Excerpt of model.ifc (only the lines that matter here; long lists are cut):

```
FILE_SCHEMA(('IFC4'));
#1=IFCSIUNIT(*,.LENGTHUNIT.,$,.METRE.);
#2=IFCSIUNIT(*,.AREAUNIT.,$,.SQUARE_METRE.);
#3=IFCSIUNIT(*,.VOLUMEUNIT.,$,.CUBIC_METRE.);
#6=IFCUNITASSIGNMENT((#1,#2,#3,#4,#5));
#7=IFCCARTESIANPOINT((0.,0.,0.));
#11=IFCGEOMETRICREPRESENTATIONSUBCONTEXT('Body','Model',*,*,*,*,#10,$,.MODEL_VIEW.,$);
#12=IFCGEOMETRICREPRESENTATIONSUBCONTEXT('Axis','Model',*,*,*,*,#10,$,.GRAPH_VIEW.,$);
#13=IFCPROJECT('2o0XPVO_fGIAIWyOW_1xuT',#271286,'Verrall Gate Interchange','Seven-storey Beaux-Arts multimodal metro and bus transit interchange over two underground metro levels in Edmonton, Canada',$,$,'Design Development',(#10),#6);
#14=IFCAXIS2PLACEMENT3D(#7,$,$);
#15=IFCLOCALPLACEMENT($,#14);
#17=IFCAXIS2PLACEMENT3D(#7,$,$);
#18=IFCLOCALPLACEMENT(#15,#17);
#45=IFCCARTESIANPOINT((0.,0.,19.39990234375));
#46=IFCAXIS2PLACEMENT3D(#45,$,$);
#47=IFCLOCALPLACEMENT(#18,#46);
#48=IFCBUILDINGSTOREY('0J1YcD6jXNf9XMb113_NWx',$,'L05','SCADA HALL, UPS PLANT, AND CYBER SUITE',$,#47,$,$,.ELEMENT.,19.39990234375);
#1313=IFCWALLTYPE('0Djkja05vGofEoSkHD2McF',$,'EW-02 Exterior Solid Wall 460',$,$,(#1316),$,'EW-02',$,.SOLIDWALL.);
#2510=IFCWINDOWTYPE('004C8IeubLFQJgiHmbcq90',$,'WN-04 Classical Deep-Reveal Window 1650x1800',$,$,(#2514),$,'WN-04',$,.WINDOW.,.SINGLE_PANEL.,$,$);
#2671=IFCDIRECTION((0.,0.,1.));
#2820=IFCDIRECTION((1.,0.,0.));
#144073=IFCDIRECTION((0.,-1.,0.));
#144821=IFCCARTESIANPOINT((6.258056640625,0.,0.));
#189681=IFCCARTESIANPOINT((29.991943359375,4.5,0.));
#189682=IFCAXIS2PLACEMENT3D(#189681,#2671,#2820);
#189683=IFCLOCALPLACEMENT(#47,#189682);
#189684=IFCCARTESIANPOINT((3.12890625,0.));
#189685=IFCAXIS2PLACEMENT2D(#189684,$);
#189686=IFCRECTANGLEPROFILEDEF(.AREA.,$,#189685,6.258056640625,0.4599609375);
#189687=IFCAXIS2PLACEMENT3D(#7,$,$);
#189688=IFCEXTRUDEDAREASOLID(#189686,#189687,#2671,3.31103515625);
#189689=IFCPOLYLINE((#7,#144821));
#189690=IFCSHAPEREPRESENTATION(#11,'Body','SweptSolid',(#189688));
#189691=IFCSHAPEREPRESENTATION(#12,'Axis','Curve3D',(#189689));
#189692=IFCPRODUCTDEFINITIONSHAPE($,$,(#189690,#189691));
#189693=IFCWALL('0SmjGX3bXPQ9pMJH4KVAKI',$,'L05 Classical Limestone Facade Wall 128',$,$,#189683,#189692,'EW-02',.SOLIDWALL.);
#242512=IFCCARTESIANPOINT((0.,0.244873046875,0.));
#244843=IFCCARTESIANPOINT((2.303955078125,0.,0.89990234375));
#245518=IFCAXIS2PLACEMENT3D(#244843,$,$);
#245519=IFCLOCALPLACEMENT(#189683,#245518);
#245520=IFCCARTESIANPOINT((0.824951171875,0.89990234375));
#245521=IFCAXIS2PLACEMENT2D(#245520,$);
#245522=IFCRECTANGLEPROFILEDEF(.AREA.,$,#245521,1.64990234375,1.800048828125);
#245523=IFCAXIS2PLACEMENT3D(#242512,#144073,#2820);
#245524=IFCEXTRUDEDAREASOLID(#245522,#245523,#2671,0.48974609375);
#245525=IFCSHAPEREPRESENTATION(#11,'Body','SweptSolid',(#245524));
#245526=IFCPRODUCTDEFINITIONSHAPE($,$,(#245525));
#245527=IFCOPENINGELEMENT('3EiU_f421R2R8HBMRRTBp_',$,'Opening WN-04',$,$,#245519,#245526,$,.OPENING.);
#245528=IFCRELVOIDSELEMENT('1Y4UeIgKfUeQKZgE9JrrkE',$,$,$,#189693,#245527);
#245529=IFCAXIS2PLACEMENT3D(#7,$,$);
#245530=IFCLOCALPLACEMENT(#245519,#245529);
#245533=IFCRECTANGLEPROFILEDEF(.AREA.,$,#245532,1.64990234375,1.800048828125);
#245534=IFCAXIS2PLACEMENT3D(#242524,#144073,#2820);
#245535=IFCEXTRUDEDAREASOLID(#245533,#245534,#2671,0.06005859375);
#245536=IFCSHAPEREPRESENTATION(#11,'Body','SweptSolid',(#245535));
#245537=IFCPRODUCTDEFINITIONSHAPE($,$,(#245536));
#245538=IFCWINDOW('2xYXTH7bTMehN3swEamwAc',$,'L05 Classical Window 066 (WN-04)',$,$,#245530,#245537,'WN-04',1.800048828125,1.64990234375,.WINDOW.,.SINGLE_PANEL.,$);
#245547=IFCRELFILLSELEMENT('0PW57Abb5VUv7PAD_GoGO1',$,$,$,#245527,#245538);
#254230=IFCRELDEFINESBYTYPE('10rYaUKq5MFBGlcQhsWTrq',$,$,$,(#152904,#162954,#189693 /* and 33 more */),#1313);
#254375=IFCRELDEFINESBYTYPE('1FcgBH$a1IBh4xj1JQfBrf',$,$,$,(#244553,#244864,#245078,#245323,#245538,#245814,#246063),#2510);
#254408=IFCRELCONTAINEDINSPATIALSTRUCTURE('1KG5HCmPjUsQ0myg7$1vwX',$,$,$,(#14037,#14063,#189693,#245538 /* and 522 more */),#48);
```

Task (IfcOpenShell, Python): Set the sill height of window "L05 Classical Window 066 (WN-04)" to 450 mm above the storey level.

```python
import numpy as np
import ifcopenshell
import ifcopenshell.api.geometry
import ifcopenshell.geom
import ifcopenshell.util.element
import ifcopenshell.util.placement
import ifcopenshell.util.shape
import ifcopenshell.util.unit

model = ifcopenshell.open("model.ifc")
unit_scale = ifcopenshell.util.unit.calculate_unit_scale(model)

window = model.by_guid("2xYXTH7bTMehN3swEamwAc")
opening = window.FillsVoids[0].RelatingOpeningElement
storey = ifcopenshell.util.element.get_container(window, ifc_class="IfcBuildingStorey")
level = ifcopenshell.util.placement.get_local_placement(storey.ObjectPlacement)[2, 3]

# The opening's origin need not be at the sill, so measure its lowest point.
shape = ifcopenshell.geom.create_shape(ifcopenshell.geom.settings(), opening)
bottom = ifcopenshell.util.shape.get_shape_bottom_elevation(shape, shape.geometry) / unit_scale
dz = level + 0.45 / unit_scale - bottom

shift = np.array([0.0, 0.0, dz])
# The window is placed relative to its opening, so it follows when the opening moves.
matrix = ifcopenshell.util.placement.get_local_placement(opening.ObjectPlacement)
matrix[:3, 3] += shift
ifcopenshell.api.geometry.edit_object_placement(
    model, product=opening, matrix=matrix, is_si=False, should_transform_children=True
)

print(f"moved by {dz * unit_scale:+.3f} m")

model.write("model_rev.ifc")
```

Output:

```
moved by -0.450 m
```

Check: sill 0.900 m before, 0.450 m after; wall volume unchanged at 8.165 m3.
